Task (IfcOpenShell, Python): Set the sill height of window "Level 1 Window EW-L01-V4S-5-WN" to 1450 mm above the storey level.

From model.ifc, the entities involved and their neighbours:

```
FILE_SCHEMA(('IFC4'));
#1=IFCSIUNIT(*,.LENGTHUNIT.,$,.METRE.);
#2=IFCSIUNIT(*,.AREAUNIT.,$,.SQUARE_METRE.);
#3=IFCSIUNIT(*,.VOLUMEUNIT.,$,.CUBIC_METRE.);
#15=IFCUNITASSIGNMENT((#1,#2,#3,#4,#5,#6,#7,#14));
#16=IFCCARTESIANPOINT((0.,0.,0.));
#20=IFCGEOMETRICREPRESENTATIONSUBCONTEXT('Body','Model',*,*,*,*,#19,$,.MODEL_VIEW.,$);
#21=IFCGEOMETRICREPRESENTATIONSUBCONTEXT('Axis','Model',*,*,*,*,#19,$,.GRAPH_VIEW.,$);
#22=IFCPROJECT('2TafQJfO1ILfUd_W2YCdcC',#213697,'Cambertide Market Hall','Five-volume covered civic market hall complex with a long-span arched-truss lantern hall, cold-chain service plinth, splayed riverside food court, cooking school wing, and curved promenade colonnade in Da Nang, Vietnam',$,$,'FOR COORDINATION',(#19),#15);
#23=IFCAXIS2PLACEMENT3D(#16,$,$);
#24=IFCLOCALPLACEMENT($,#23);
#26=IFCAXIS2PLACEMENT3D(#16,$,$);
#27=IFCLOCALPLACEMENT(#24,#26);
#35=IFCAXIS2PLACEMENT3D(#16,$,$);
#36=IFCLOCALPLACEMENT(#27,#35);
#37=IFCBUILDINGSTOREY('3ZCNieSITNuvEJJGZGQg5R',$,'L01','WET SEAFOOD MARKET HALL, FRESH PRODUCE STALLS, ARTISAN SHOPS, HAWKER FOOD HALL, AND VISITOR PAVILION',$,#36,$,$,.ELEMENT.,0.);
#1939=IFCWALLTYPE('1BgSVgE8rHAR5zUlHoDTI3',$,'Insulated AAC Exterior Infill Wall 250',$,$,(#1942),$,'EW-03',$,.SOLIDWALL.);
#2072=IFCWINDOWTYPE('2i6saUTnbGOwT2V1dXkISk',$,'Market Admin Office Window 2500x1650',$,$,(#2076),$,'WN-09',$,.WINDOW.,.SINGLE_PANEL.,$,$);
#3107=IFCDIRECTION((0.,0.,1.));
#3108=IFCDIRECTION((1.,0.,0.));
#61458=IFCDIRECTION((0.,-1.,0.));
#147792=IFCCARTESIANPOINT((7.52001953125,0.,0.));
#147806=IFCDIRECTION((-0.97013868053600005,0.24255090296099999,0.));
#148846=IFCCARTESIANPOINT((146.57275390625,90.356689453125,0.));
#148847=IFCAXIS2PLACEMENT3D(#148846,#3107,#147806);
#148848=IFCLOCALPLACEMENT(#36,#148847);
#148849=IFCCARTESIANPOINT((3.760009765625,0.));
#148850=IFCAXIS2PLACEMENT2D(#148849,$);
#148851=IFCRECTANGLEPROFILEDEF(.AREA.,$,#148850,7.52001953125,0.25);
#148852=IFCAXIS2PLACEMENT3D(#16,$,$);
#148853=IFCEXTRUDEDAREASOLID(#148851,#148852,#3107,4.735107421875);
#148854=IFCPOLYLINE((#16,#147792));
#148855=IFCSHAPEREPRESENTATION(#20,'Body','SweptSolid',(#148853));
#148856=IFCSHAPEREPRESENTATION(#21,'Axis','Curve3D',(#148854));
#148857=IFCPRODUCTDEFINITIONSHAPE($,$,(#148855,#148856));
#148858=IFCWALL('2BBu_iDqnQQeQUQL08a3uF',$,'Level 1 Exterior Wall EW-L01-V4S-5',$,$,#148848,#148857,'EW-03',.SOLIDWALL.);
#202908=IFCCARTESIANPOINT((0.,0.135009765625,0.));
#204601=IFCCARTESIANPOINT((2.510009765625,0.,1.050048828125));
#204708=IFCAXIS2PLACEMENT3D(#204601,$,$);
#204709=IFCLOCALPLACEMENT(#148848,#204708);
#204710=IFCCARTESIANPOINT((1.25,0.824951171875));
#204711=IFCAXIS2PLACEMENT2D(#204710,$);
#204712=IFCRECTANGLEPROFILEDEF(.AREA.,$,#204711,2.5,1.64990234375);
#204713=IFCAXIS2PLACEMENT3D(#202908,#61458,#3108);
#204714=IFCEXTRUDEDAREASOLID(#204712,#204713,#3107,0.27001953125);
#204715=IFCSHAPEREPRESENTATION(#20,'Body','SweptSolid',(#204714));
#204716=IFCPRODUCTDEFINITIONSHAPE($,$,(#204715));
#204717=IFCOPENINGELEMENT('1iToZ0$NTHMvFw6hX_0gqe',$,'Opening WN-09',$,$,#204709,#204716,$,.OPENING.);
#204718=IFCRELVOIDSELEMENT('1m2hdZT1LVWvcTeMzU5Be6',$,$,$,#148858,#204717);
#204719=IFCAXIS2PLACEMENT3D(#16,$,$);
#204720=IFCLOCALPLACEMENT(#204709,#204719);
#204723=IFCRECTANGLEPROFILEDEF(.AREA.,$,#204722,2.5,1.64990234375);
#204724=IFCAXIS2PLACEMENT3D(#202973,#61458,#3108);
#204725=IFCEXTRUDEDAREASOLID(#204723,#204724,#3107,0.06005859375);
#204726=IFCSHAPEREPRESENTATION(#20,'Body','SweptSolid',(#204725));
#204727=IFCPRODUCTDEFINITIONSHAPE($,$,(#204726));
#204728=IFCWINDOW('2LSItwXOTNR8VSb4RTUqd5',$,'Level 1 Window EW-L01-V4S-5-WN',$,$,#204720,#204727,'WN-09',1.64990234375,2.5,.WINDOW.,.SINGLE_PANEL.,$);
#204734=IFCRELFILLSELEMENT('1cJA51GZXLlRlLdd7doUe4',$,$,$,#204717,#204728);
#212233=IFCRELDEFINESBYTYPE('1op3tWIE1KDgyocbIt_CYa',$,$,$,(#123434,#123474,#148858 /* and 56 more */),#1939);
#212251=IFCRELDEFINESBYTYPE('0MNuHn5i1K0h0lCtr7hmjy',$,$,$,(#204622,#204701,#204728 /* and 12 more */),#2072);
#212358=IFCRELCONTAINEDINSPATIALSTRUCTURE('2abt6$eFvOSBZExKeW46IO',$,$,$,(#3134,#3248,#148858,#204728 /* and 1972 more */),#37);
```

```python
import numpy as np
import ifcopenshell
import ifcopenshell.api.geometry
import ifcopenshell.geom
import ifcopenshell.util.element
import ifcopenshell.util.placement
import ifcopenshell.util.shape
import ifcopenshell.util.unit

model = ifcopenshell.open("model.ifc")
unit_scale = ifcopenshell.util.unit.calculate_unit_scale(model)

window = model.by_guid("2LSItwXOTNR8VSb4RTUqd5")
opening = window.FillsVoids[0].RelatingOpeningElement
storey = ifcopenshell.util.element.get_container(window, ifc_class="IfcBuildingStorey")
level = ifcopenshell.util.placement.get_local_placement(storey.ObjectPlacement)[2, 3]

# The opening's origin need not be at the sill, so measure its lowest point.
shape = ifcopenshell.geom.create_shape(ifcopenshell.geom.settings(), opening)
bottom = ifcopenshell.util.shape.get_shape_bottom_elevation(shape, shape.geometry) / unit_scale
dz = level + 1.45 - bottom

shift = np.array([0.0, 0.0, dz])
# The window is placed relative to its opening, so it follows when the opening moves.
matrix = ifcopenshell.util.placement.get_local_placement(opening.ObjectPlacement)
matrix[:3, 3] += shift
ifcopenshell.api.geometry.edit_object_placement(
    model, product=opening, matrix=matrix, is_si=False, should_transform_children=True
)

print(f"moved by {dz * unit_scale:+.3f} m")

model.write("model_updated.ifc")
```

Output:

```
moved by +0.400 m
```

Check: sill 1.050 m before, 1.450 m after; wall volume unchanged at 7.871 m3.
